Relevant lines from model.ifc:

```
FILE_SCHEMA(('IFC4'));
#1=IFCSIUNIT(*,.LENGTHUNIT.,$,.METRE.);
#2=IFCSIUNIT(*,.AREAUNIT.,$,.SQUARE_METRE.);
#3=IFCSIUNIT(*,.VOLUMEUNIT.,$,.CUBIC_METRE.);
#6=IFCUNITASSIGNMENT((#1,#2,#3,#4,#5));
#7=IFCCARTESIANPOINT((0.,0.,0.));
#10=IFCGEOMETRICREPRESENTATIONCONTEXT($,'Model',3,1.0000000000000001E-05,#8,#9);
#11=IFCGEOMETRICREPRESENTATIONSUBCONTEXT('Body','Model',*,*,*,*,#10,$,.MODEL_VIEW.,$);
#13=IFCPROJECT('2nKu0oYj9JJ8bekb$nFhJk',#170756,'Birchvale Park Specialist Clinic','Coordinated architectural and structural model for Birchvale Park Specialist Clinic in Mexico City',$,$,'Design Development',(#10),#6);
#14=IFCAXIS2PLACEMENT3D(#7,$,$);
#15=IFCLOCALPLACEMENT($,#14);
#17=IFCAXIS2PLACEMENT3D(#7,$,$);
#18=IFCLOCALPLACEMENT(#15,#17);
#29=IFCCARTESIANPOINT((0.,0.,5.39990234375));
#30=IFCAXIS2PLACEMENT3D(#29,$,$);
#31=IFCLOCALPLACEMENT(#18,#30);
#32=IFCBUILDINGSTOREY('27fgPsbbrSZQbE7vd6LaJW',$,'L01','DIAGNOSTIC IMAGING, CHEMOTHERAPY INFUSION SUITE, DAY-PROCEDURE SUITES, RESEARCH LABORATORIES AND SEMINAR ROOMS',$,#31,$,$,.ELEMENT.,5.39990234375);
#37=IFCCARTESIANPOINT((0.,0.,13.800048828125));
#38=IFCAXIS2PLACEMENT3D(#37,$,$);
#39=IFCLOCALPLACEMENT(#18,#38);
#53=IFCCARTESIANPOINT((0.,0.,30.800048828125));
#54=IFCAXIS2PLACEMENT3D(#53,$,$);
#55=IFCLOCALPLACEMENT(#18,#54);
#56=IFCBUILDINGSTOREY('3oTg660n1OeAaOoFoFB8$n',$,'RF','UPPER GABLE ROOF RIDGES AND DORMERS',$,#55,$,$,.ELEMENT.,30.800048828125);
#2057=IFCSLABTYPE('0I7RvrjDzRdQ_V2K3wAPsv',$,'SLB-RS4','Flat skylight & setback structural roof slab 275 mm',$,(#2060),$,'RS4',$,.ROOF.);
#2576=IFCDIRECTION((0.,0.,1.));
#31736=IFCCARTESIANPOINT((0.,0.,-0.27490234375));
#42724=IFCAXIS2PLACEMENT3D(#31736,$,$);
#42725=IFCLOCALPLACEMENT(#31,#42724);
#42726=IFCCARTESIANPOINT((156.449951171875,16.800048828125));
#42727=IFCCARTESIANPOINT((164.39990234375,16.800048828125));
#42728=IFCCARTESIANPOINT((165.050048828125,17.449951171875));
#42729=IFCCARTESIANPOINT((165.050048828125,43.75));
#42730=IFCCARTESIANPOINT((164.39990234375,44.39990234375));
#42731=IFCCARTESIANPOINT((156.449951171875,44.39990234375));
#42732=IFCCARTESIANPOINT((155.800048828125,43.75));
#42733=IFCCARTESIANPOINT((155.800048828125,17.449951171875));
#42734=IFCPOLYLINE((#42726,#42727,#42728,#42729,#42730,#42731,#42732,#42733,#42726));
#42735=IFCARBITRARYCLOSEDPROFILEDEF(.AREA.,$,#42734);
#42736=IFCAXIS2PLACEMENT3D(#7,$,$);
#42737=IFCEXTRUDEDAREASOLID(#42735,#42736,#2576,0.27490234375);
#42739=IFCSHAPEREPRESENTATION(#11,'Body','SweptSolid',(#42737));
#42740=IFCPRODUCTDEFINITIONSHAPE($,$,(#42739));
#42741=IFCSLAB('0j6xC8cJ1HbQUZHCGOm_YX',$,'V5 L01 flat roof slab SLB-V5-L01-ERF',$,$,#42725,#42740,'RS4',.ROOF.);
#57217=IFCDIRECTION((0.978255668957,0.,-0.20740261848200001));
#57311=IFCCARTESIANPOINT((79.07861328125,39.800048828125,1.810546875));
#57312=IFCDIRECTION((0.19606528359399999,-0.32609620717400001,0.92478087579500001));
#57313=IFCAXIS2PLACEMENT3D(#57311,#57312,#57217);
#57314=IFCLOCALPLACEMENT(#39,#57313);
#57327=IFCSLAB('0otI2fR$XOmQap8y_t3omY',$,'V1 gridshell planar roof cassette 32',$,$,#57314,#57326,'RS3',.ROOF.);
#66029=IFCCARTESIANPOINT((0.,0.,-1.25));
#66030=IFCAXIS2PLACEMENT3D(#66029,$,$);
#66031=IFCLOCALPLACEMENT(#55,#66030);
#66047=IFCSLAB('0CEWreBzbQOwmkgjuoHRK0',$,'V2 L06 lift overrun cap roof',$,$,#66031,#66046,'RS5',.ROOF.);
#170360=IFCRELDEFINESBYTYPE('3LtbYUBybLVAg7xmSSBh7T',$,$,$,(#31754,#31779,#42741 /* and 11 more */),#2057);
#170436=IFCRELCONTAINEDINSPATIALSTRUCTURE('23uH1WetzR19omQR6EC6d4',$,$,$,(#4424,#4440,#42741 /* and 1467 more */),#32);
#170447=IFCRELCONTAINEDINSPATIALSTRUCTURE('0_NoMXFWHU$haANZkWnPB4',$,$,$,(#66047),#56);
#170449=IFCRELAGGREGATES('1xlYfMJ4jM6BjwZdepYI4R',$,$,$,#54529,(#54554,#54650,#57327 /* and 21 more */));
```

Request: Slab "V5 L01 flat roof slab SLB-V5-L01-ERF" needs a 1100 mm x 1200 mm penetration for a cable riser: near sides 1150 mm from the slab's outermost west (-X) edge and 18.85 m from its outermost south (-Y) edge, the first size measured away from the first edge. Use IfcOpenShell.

```python
import numpy as np
import ifcopenshell
import ifcopenshell.api.feature
import ifcopenshell.api.geometry
import ifcopenshell.api.root
import ifcopenshell.geom
import ifcopenshell.util.placement
import ifcopenshell.util.representation
import ifcopenshell.util.shape
import ifcopenshell.util.unit

model = ifcopenshell.open("model.ifc")
unit_scale = ifcopenshell.util.unit.calculate_unit_scale(model)
settings = ifcopenshell.geom.settings()


def volume(element):
    """Net volume in cubic metres, openings subtracted."""
    shape = ifcopenshell.geom.create_shape(settings, element)
    return ifcopenshell.util.shape.get_volume(shape.geometry)


slab = model.by_guid("0j6xC8cJ1HbQUZHCGOm_YX")
before = volume(slab)

# Extent in the slab's own axes, in metres. The edges named are its -X and -Y sides.
slab_shape = ifcopenshell.geom.create_shape(settings, slab)
vertices = ifcopenshell.util.shape.get_vertices(slab_shape.geometry)
x_min, y_min, bottom = vertices.min(axis=0)
top = vertices[:, 2].max()

opening = ifcopenshell.api.root.create_entity(model, ifc_class="IfcOpeningElement", name="Cable riser opening", predefined_type="OPENING")
context = ifcopenshell.util.representation.get_context(model, "Model", "Body", "MODEL_VIEW")
width, depth = 1.1, 1.2
outline = [(0.0, 0.0), (width, 0.0), (width, depth), (0.0, depth), (0.0, 0.0)]
# Overshoot both faces by 50 mm so the cut is clean.
shape = ifcopenshell.api.geometry.add_slab_representation(
    model, context=context, depth=top - bottom + 0.1, polyline=outline
)
ifcopenshell.api.geometry.assign_representation(model, product=opening, representation=shape)

matrix = ifcopenshell.util.placement.get_local_placement(slab.ObjectPlacement)
matrix[:, 3] = matrix @ np.append(np.array([x_min + 1.15, y_min + 18.85, bottom - 0.05]) / unit_scale, 1.0)
ifcopenshell.api.geometry.edit_object_placement(model, product=opening, matrix=matrix, is_si=False)
ifcopenshell.api.feature.add_feature(model, feature=opening, element=slab)

after = volume(slab)

print(f"slab volume {before:.3f} -> {after:.3f} m3")

model.write("model_updated.ifc")
```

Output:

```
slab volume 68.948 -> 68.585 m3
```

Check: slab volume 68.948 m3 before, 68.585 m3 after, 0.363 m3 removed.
